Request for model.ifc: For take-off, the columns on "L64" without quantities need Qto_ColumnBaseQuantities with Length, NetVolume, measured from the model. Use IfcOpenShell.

First a look at what the model holds.

```python
import ifcopenshell
import ifcopenshell.util.element
import ifcopenshell.util.unit

model = ifcopenshell.open("model.ifc")
print(model.schema)
for unit_type in ("LENGTHUNIT", "AREAUNIT", "VOLUMEUNIT"):
    print(unit_type, ifcopenshell.util.unit.calculate_unit_scale(model, unit_type))
storey = next(s for s in model.by_type("IfcBuildingStorey") if s.Name == "L64")
columns = [e for e in ifcopenshell.util.element.get_decomposition(storey) if e.is_a("IfcColumn")]
for e in sorted(columns, key=lambda e: e.id()):
    print(e.id(), e.is_a(), e.Name, list(ifcopenshell.util.element.get_psets(e, qtos_only=True)), sep=" | ")
```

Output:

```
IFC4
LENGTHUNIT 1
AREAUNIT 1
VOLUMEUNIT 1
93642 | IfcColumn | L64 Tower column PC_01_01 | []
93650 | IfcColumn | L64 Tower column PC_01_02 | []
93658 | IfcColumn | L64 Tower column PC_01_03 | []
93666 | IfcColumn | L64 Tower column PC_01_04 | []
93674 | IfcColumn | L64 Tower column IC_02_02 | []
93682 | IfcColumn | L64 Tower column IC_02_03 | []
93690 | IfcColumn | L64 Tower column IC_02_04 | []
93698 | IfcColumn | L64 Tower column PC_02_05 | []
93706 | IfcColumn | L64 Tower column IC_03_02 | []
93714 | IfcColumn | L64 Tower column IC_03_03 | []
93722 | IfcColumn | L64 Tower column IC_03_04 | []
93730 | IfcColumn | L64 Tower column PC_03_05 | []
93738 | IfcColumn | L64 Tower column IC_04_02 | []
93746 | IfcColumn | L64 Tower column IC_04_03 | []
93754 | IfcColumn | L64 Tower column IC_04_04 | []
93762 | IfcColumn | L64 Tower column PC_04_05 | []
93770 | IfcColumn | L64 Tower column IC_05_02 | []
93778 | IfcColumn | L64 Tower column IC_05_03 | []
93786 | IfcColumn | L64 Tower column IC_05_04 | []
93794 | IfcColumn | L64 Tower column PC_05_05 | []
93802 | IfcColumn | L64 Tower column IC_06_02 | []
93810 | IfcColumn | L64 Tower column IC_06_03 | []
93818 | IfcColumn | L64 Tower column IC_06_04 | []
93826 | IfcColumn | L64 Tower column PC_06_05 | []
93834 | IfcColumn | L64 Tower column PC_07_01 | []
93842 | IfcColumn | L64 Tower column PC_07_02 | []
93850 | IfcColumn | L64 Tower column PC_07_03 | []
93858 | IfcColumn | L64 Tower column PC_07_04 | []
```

```python
import ifcopenshell
import ifcopenshell.api.pset
import ifcopenshell.geom
import ifcopenshell.util.element
import ifcopenshell.util.shape
import ifcopenshell.util.unit

model = ifcopenshell.open("model.ifc")
unit_scale = ifcopenshell.util.unit.calculate_unit_scale(model)
volume_scale = ifcopenshell.util.unit.calculate_unit_scale(model, "VOLUMEUNIT")
settings = ifcopenshell.geom.settings()

storey = next(s for s in model.by_type("IfcBuildingStorey") if s.Name == "L64")
columns = [e for e in ifcopenshell.util.element.get_decomposition(storey) if e.is_a("IfcColumn")]

for e in sorted(columns, key=lambda e: e.id()):
    if ifcopenshell.util.element.get_psets(e, qtos_only=True, should_inherit=False):
        continue
    # Geometry comes back in metres, in the element's own axes.
    shape = ifcopenshell.geom.create_shape(settings, e)
    values = {
        "Length": ifcopenshell.util.shape.get_z(shape.geometry) / unit_scale,
        "NetVolume": ifcopenshell.util.shape.get_volume(shape.geometry) / volume_scale,
    }
    qto = ifcopenshell.api.pset.add_qto(model, product=e, name="Qto_ColumnBaseQuantities")
    ifcopenshell.api.pset.edit_qto(model, qto=qto, properties=values)
    print(e.id(), {k: round(v, 3) for k, v in values.items()})

model.write("model-out.ifc")
```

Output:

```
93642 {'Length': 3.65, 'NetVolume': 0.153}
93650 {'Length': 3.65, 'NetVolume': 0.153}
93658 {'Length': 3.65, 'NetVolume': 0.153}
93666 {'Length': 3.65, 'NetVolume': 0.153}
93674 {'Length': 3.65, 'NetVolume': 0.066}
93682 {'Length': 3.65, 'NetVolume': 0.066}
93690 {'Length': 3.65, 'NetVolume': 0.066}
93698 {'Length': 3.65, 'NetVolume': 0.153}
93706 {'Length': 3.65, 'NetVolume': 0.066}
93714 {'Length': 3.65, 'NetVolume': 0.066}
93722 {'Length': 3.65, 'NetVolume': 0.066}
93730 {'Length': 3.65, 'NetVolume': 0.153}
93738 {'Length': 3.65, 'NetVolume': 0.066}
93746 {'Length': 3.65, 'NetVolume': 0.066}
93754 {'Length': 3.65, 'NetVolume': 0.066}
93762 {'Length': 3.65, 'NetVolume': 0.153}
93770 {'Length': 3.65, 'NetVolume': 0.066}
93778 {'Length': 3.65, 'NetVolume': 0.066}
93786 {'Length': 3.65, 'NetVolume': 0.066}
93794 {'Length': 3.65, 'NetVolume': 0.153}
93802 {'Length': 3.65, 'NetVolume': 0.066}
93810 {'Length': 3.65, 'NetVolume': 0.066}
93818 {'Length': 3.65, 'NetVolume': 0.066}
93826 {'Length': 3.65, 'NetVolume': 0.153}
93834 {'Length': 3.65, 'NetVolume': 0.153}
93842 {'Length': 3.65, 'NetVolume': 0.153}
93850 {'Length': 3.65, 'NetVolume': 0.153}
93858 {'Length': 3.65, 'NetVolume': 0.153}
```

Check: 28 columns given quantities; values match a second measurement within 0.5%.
